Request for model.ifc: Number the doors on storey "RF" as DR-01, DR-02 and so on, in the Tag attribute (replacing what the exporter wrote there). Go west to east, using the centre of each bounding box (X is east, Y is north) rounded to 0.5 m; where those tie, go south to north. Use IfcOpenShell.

First a look at what the model holds.

```python
import ifcopenshell
import ifcopenshell.util.element
import ifcopenshell.util.placement

model = ifcopenshell.open("model.ifc")
print(model.schema)
storey = next(s for s in model.by_type("IfcBuildingStorey") if s.Name == "RF")
doors = [e for e in ifcopenshell.util.element.get_decomposition(storey) if e.is_a("IfcDoor")]
for e in sorted(doors, key=lambda e: e.id()):
    origin = ifcopenshell.util.placement.get_local_placement(e.ObjectPlacement)[:3, 3]
    print(e.id(), e.Tag, e.Name, origin.round(2) + 0.0, sep=" | ")
```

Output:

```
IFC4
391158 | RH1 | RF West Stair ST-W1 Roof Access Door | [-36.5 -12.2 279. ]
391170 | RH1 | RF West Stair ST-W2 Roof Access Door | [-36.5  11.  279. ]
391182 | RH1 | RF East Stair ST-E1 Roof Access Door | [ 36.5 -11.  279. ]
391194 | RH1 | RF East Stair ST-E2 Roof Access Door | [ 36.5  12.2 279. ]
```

```python
import ifcopenshell
import ifcopenshell.geom
import ifcopenshell.util.element
import ifcopenshell.util.shape

model = ifcopenshell.open("model.ifc")
settings = ifcopenshell.geom.settings()
settings.set("use-world-coords", True)


def centre(element):
    shape = ifcopenshell.geom.create_shape(settings, element)
    return ifcopenshell.util.shape.get_bbox_centroid(shape.geometry)


storey = next(s for s in model.by_type("IfcBuildingStorey") if s.Name == "RF")
doors = [e for e in ifcopenshell.util.element.get_decomposition(storey) if e.is_a("IfcDoor")]

# Insertion points can sit at a corner or the storey origin, so sort by the geometry (in metres).
centres = {e: centre(e) for e in doors}
doors.sort(key=lambda e: (round(centres[e][0] / 0.5), centres[e][1]))

for i, e in enumerate(doors, start=1):
    number = f"DR-{i:02d}"
    e.Tag = number
    print(e.id(), number)

model.write("model_updated.ifc")
```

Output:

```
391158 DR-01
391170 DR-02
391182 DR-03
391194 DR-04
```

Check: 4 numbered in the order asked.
